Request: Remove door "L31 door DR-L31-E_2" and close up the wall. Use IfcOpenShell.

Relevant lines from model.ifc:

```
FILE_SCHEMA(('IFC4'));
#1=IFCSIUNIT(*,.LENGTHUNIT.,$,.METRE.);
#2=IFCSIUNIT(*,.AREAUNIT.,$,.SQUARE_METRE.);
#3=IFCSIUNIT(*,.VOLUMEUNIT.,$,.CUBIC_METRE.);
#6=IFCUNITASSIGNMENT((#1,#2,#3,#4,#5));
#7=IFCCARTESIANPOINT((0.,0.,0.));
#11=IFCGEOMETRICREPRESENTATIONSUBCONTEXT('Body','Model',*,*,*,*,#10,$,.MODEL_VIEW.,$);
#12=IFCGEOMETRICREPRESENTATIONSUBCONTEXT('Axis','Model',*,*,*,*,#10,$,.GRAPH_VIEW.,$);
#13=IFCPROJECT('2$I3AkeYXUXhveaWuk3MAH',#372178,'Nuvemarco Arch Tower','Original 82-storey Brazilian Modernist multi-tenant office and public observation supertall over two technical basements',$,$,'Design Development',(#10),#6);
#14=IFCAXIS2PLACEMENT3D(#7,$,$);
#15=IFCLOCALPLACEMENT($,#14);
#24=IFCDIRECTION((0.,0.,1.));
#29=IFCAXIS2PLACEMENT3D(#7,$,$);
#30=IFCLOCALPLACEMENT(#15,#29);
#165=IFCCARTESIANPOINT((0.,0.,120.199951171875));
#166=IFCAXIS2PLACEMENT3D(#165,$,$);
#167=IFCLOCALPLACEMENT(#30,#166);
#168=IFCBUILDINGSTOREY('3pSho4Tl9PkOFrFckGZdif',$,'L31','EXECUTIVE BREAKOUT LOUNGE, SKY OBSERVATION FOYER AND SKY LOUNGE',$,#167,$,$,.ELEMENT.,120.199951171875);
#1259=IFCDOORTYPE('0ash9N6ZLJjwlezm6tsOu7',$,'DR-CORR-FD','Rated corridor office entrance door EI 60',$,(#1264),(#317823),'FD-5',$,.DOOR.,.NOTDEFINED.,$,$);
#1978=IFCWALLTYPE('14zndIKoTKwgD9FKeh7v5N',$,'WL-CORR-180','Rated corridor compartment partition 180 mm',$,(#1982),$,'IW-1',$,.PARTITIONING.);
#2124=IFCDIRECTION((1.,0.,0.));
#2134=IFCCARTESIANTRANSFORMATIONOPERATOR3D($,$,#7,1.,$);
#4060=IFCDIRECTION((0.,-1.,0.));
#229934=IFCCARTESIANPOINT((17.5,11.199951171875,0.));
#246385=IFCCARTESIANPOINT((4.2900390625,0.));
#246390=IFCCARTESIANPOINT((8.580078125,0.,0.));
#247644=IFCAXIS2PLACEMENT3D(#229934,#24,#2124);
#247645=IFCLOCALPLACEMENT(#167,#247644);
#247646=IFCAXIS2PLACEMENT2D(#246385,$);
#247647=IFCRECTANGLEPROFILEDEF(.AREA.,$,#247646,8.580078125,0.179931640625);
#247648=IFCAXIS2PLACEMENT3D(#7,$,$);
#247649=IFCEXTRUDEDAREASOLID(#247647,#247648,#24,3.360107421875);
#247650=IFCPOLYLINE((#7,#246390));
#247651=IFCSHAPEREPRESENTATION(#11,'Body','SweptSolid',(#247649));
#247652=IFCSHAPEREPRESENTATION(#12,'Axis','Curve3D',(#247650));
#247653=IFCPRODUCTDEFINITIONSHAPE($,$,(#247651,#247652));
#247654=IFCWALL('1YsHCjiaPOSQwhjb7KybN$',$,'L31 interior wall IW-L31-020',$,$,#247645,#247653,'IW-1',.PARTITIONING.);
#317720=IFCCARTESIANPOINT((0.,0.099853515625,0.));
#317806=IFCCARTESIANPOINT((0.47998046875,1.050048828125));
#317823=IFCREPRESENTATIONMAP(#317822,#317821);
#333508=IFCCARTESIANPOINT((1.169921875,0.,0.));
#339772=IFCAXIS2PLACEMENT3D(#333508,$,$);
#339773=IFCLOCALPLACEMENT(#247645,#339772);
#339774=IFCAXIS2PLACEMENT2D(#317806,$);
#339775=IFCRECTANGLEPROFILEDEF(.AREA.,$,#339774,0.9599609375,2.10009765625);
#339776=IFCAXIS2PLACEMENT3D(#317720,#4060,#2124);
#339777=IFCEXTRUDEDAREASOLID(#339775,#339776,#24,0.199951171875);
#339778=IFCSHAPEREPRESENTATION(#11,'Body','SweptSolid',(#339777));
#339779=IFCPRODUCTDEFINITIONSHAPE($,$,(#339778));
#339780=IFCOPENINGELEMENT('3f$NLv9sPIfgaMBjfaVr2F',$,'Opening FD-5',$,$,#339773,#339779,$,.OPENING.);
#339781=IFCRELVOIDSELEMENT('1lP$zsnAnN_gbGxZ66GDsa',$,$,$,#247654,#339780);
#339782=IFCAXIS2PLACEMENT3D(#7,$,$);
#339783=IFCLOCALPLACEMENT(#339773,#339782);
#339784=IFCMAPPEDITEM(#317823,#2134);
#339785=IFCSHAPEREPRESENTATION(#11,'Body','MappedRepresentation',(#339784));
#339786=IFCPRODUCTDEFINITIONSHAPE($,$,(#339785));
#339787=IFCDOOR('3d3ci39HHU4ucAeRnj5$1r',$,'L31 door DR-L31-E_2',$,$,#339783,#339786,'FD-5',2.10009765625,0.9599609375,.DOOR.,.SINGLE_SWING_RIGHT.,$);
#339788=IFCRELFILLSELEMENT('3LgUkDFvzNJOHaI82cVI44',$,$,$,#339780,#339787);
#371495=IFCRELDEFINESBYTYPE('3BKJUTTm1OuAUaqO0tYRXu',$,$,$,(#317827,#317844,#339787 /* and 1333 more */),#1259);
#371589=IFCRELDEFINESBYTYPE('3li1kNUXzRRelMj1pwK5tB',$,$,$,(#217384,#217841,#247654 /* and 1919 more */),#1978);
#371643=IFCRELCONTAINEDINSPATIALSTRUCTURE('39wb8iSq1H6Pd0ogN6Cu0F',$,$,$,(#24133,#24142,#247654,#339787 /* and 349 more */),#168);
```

```python
import ifcopenshell
import ifcopenshell.api.feature
import ifcopenshell.api.root
import ifcopenshell.geom
import ifcopenshell.util.shape

model = ifcopenshell.open("model.ifc")
settings = ifcopenshell.geom.settings()


def volume(element):
    """Net volume in cubic metres, openings subtracted."""
    shape = ifcopenshell.geom.create_shape(settings, element)
    return ifcopenshell.util.shape.get_volume(shape.geometry)


door = model.by_guid("3d3ci39HHU4ucAeRnj5$1r")
opening = door.FillsVoids[0].RelatingOpeningElement
wall = opening.VoidsElements[0].RelatingBuildingElement
before = volume(wall)

ifcopenshell.api.root.remove_product(model, product=door)
ifcopenshell.api.feature.remove_feature(model, feature=opening)

after = volume(wall)

print(f"wall volume {before:.3f} -> {after:.3f} m3")

model.write("model_rev.ifc")
```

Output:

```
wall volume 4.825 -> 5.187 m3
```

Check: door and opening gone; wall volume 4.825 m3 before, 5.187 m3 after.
